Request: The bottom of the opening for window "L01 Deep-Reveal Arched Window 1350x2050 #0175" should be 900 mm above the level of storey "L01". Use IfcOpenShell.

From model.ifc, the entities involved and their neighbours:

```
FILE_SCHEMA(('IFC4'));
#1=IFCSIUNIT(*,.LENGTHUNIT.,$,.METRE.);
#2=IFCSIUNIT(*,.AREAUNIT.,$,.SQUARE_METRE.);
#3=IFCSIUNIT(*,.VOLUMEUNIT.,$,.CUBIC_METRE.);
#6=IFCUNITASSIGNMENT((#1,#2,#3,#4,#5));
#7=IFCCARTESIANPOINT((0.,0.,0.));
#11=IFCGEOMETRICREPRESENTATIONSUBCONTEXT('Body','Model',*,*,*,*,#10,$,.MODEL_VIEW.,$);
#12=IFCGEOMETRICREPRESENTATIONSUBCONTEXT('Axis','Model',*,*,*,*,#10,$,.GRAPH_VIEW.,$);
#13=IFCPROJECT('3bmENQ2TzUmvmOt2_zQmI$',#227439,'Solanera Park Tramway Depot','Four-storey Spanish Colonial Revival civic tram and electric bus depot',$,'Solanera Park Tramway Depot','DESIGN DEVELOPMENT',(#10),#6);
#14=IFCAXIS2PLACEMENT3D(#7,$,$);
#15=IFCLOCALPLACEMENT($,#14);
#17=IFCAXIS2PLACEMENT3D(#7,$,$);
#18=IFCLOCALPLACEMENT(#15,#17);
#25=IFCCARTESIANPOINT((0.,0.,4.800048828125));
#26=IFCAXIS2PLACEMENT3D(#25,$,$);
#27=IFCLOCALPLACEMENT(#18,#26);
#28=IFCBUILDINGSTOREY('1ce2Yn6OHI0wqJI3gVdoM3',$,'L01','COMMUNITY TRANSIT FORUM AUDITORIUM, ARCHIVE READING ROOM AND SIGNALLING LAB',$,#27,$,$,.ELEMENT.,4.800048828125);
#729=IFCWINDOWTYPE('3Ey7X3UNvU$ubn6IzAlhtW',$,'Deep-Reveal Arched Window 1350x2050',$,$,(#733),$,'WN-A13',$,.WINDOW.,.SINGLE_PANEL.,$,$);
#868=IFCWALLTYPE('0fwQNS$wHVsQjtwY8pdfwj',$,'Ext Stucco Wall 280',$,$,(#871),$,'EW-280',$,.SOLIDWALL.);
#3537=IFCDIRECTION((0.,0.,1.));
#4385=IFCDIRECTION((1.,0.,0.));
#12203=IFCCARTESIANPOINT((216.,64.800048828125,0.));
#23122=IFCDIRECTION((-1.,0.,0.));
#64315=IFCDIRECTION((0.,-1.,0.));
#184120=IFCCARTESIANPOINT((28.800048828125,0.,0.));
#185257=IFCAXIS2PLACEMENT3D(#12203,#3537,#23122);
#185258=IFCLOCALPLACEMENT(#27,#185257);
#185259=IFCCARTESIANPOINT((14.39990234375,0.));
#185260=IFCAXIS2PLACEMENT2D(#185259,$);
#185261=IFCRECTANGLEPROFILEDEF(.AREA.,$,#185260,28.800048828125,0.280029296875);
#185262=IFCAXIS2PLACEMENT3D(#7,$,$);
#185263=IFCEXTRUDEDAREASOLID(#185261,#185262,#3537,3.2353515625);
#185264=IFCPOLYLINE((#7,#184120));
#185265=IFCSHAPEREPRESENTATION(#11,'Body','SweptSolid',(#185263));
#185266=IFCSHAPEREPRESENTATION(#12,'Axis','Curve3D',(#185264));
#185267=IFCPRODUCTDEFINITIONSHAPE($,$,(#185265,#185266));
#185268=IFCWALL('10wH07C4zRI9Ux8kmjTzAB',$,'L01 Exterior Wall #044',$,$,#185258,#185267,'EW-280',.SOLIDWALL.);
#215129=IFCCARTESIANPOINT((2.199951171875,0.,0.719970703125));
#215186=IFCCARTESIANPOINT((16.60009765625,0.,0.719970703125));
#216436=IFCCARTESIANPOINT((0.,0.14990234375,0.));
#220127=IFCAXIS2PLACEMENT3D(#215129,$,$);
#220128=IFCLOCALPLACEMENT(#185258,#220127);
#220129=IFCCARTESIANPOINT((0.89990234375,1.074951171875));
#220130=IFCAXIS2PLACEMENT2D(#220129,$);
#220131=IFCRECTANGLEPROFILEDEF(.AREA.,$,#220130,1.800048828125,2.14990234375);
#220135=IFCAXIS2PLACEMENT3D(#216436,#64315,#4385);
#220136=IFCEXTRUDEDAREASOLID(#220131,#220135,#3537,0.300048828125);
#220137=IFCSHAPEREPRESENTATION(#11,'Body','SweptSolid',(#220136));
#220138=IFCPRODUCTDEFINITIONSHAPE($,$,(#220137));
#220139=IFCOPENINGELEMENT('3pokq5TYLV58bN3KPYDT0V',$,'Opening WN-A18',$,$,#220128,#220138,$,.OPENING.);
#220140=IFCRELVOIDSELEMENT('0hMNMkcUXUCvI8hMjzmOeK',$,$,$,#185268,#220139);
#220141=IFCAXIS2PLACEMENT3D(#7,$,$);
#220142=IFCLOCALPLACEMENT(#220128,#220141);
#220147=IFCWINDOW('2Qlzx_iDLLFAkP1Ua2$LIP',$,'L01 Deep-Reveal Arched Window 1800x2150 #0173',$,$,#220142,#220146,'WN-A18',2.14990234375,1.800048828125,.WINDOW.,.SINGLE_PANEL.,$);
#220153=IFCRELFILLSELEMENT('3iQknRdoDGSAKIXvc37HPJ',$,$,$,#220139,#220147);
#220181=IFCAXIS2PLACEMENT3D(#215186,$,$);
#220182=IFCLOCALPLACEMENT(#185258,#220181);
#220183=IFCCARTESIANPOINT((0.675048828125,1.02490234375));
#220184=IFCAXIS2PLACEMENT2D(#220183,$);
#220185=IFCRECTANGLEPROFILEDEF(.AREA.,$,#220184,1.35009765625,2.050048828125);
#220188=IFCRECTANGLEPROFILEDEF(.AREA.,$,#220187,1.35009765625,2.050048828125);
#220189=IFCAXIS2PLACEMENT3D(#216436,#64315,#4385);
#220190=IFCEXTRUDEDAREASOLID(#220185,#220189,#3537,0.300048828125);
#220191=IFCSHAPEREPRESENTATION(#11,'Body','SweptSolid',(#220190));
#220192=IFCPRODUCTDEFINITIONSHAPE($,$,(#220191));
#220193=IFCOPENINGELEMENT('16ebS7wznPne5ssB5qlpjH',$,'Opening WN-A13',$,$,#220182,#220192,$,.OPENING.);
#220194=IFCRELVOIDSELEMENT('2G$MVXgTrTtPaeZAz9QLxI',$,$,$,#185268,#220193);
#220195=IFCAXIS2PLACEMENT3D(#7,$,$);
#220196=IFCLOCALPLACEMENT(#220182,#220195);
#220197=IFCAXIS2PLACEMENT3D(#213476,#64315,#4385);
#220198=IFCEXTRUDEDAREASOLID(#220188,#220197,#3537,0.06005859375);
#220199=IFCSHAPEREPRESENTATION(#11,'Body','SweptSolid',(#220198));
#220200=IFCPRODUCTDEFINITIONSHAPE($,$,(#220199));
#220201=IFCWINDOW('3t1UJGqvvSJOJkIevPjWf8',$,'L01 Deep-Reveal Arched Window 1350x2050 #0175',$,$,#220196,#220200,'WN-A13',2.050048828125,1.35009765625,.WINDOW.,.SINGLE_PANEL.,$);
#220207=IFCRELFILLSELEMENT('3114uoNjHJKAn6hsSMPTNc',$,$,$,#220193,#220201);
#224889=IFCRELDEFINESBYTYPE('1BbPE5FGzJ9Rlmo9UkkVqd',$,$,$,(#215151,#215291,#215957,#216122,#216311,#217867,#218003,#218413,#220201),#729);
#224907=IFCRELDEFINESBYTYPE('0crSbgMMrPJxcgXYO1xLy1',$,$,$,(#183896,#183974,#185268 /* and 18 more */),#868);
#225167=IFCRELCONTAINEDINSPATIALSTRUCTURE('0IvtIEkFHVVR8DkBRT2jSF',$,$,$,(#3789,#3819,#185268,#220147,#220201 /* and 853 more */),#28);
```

```python
import numpy as np
import ifcopenshell
import ifcopenshell.api.geometry
import ifcopenshell.geom
import ifcopenshell.util.element
import ifcopenshell.util.placement
import ifcopenshell.util.shape
import ifcopenshell.util.unit

model = ifcopenshell.open("model.ifc")
unit_scale = ifcopenshell.util.unit.calculate_unit_scale(model)

window = model.by_id(220201)
opening = window.FillsVoids[0].RelatingOpeningElement
storey = ifcopenshell.util.element.get_container(window, ifc_class="IfcBuildingStorey")
level = ifcopenshell.util.placement.get_local_placement(storey.ObjectPlacement)[2, 3]

# The opening's origin need not be at the sill, so measure its lowest point.
shape = ifcopenshell.geom.create_shape(ifcopenshell.geom.settings(), opening)
bottom = ifcopenshell.util.shape.get_shape_bottom_elevation(shape, shape.geometry) / unit_scale
dz = level + 0.9 - bottom

shift = np.array([0.0, 0.0, dz])
# The window is placed relative to its opening, so it follows when the opening moves.
matrix = ifcopenshell.util.placement.get_local_placement(opening.ObjectPlacement)
matrix[:3, 3] += shift
ifcopenshell.api.geometry.edit_object_placement(
    model, product=opening, matrix=matrix, is_si=False, should_transform_children=True
)

print(f"moved by {dz * unit_scale:+.3f} m")

model.write("model_updated.ifc")
```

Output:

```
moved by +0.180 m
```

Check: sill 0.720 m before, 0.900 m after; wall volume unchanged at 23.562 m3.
